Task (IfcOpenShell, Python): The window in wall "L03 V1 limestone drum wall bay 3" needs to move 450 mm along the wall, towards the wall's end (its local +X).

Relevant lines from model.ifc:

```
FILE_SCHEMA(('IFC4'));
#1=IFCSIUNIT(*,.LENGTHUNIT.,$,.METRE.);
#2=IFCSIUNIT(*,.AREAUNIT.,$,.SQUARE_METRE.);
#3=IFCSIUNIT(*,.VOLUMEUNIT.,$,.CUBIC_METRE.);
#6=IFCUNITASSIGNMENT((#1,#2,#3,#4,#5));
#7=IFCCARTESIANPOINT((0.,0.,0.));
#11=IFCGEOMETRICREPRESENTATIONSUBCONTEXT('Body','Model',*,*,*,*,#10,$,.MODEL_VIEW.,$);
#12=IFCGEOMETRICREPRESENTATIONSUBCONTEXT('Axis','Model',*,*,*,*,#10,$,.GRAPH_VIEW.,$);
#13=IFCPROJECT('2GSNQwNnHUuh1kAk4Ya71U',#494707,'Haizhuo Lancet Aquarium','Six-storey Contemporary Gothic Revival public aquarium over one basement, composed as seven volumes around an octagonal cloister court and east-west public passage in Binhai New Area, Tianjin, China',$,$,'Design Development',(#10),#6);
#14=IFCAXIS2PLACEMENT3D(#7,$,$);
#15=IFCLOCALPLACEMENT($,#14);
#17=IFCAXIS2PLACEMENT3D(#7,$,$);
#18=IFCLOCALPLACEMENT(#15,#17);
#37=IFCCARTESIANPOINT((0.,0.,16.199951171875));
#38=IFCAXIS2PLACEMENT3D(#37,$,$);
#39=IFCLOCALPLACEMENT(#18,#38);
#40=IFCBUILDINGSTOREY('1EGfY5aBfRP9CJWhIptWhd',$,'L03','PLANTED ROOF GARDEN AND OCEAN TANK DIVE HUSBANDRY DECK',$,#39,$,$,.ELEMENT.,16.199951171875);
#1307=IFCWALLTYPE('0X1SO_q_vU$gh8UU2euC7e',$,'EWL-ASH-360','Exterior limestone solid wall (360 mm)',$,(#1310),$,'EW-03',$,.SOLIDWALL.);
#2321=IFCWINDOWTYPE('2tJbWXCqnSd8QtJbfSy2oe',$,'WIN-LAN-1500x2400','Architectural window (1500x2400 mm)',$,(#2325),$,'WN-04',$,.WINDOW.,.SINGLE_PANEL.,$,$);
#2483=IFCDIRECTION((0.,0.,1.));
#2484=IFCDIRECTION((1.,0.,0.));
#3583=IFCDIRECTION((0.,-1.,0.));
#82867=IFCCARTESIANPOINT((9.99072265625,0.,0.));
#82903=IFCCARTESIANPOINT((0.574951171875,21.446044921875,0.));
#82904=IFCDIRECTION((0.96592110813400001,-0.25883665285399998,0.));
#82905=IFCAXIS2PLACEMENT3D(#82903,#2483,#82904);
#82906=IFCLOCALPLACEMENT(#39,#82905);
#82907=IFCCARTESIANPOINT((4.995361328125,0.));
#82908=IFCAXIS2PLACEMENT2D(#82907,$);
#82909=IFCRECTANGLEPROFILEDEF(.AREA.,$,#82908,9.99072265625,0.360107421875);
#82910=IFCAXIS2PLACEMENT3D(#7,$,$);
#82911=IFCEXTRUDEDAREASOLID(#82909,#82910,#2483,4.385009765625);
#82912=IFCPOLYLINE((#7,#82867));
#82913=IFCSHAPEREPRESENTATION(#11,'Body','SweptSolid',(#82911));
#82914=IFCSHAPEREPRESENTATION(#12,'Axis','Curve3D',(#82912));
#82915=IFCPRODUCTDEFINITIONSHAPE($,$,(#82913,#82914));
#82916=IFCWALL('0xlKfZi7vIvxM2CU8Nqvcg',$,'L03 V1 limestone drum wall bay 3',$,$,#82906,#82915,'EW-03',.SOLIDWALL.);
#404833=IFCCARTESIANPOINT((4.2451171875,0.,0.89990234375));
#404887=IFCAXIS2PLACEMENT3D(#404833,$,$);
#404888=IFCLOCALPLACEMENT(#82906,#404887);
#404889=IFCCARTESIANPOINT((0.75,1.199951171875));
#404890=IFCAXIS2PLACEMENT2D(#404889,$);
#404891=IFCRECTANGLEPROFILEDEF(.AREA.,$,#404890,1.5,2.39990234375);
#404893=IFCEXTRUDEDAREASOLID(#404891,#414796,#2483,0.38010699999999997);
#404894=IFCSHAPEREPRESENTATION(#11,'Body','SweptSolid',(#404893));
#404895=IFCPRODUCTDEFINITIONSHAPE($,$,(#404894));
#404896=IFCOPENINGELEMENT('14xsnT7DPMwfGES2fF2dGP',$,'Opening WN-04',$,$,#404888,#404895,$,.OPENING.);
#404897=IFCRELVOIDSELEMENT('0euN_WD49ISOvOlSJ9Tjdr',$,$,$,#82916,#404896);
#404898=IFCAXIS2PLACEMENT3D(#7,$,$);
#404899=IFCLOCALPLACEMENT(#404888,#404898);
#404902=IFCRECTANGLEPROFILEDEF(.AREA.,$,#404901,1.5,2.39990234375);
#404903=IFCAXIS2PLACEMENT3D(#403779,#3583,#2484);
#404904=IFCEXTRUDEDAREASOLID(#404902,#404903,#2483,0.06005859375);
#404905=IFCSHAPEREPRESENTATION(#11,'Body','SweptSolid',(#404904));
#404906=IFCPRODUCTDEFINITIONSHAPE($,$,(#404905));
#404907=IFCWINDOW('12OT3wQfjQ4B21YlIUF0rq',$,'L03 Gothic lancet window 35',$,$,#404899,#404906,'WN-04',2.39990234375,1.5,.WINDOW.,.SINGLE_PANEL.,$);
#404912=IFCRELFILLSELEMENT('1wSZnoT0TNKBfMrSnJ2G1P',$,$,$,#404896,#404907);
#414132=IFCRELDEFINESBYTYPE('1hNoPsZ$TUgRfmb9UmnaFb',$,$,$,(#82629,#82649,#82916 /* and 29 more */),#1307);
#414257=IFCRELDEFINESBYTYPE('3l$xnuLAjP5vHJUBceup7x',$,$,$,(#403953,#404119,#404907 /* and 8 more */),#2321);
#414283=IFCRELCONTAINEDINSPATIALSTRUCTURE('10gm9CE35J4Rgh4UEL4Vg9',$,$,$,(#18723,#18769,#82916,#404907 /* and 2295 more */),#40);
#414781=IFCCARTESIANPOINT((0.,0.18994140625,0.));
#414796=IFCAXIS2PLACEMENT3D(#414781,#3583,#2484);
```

```python
import ifcopenshell
import ifcopenshell.api.geometry
import ifcopenshell.util.placement

model = ifcopenshell.open("model.ifc")

window = model.by_guid("12OT3wQfjQ4B21YlIUF0rq")
opening = window.FillsVoids[0].RelatingOpeningElement
wall = opening.VoidsElements[0].RelatingBuildingElement

wall_matrix = ifcopenshell.util.placement.get_local_placement(wall.ObjectPlacement)
shift = wall_matrix[:3, 0] * 0.45
before = ifcopenshell.util.placement.get_local_placement(window.ObjectPlacement)[:3, 3].copy()

# The window is placed relative to its opening, so it follows when the opening moves.
matrix = ifcopenshell.util.placement.get_local_placement(opening.ObjectPlacement)
matrix[:3, 3] += shift
ifcopenshell.api.geometry.edit_object_placement(
    model, product=opening, matrix=matrix, is_si=False, should_transform_children=True
)

after = ifcopenshell.util.placement.get_local_placement(window.ObjectPlacement)[:3, 3]
print("window moved by", (after - before).round(3) + 0.0)

model.write("model_edited.ifc")
```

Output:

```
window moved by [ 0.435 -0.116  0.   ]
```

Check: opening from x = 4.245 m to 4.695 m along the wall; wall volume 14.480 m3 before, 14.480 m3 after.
